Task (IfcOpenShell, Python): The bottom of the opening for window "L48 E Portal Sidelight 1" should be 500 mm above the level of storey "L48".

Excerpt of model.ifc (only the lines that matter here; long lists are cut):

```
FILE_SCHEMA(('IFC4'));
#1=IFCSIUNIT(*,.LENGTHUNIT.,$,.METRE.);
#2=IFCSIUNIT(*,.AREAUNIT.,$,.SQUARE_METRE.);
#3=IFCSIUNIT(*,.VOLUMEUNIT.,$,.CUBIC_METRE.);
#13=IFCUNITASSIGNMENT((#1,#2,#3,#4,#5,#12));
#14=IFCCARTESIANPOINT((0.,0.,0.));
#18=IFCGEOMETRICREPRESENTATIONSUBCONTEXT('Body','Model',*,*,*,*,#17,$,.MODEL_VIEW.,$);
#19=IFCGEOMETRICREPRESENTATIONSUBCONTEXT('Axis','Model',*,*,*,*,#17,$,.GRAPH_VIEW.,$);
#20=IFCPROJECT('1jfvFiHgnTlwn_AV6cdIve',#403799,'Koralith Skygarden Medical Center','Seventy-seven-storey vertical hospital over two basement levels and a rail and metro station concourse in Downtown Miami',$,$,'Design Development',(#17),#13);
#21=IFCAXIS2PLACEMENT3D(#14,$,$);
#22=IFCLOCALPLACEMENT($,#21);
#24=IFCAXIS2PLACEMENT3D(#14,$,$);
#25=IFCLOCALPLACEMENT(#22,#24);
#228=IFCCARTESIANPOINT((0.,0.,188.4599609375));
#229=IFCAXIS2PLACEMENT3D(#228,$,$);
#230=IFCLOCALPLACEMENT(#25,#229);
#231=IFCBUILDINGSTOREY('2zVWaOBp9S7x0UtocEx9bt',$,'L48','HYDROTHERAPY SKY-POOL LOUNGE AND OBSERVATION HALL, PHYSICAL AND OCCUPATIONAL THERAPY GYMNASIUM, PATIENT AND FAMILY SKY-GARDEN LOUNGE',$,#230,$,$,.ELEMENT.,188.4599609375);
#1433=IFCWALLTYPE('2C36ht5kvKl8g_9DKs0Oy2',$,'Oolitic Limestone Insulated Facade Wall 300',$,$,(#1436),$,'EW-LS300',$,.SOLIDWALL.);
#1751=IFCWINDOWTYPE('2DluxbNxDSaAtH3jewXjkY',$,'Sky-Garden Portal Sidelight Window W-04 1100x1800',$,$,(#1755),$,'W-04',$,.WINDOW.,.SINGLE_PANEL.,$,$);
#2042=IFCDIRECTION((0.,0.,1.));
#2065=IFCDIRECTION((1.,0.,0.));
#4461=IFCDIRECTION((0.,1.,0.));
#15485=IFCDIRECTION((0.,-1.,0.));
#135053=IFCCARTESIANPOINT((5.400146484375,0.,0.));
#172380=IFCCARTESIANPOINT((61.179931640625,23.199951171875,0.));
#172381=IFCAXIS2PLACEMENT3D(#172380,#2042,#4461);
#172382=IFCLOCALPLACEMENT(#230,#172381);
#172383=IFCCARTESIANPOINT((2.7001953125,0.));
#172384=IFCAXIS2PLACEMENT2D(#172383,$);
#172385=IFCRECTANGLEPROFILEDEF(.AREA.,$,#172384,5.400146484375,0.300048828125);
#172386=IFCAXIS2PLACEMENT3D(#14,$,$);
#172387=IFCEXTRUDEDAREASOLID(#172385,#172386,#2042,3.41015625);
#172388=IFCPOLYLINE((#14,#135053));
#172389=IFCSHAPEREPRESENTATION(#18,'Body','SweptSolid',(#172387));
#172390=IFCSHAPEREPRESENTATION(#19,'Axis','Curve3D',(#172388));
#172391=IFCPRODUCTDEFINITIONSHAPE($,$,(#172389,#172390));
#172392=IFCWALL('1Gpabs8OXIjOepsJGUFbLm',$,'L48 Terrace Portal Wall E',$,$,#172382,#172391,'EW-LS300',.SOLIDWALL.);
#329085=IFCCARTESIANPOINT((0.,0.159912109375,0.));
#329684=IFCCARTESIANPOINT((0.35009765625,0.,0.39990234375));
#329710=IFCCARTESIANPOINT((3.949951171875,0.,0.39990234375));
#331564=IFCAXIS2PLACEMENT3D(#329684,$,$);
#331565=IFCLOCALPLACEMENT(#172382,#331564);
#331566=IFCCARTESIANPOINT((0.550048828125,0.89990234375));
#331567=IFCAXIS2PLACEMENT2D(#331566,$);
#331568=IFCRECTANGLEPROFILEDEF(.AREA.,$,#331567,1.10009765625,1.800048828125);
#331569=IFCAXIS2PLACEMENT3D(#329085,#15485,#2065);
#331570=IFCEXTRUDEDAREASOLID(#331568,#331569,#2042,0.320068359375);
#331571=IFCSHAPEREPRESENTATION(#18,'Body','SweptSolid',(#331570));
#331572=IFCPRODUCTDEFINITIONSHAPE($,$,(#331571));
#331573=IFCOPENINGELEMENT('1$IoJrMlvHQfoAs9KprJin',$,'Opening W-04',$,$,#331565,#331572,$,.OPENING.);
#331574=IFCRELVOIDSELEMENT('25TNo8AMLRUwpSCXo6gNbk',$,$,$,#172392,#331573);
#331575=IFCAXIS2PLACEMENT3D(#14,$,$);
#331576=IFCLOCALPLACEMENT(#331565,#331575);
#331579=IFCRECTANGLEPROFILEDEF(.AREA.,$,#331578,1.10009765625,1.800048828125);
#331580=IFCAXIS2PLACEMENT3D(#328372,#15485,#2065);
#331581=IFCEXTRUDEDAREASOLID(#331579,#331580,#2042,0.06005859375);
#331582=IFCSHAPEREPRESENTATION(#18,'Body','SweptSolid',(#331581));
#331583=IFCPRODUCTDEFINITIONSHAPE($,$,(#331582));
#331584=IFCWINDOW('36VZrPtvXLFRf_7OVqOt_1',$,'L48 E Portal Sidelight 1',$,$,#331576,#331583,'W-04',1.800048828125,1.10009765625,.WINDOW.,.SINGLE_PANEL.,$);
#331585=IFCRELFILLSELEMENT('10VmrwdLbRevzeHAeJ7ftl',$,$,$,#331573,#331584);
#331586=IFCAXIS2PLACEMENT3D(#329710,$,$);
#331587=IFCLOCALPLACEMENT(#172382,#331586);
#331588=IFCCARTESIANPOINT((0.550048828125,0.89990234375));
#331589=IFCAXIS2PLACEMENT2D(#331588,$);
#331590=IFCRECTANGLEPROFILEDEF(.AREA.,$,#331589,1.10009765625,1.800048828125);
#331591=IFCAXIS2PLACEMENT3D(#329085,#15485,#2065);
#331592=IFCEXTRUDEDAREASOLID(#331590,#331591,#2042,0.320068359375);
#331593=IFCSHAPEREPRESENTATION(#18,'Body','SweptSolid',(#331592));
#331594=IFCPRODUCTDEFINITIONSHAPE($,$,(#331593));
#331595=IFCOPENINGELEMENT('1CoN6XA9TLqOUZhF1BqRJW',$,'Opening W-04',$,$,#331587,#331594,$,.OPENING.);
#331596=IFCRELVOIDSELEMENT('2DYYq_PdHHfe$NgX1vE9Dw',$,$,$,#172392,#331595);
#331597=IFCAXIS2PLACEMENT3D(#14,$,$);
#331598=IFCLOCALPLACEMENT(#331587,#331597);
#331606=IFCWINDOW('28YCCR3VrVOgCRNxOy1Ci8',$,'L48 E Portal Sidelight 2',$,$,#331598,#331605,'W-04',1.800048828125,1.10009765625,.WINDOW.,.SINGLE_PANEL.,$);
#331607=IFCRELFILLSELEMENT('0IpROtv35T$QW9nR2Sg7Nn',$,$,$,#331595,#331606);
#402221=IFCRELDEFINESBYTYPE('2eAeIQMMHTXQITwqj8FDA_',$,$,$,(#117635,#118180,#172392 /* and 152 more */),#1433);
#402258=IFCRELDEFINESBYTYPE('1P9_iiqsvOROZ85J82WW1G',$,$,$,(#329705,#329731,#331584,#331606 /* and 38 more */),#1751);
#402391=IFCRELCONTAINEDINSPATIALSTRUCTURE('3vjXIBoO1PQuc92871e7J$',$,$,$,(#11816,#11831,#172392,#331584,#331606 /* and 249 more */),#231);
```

```python
import numpy as np
import ifcopenshell
import ifcopenshell.api.geometry
import ifcopenshell.geom
import ifcopenshell.util.element
import ifcopenshell.util.placement
import ifcopenshell.util.shape
import ifcopenshell.util.unit

model = ifcopenshell.open("model.ifc")
unit_scale = ifcopenshell.util.unit.calculate_unit_scale(model)

window = model.by_guid("36VZrPtvXLFRf_7OVqOt_1")
opening = window.FillsVoids[0].RelatingOpeningElement
storey = ifcopenshell.util.element.get_container(window, ifc_class="IfcBuildingStorey")
level = ifcopenshell.util.placement.get_local_placement(storey.ObjectPlacement)[2, 3]

# The opening's origin need not be at the sill, so measure its lowest point.
shape = ifcopenshell.geom.create_shape(ifcopenshell.geom.settings(), opening)
bottom = ifcopenshell.util.shape.get_shape_bottom_elevation(shape, shape.geometry) / unit_scale
dz = level + 0.5 / unit_scale - bottom

shift = np.array([0.0, 0.0, dz])
# The window is placed relative to its opening, so it follows when the opening moves.
matrix = ifcopenshell.util.placement.get_local_placement(opening.ObjectPlacement)
matrix[:3, 3] += shift
ifcopenshell.api.geometry.edit_object_placement(
    model, product=opening, matrix=matrix, is_si=False, should_transform_children=True
)

print(f"moved by {dz * unit_scale:+.3f} m")

model.write("model_v2.ifc")
```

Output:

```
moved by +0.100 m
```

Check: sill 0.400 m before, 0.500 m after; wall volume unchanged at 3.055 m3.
